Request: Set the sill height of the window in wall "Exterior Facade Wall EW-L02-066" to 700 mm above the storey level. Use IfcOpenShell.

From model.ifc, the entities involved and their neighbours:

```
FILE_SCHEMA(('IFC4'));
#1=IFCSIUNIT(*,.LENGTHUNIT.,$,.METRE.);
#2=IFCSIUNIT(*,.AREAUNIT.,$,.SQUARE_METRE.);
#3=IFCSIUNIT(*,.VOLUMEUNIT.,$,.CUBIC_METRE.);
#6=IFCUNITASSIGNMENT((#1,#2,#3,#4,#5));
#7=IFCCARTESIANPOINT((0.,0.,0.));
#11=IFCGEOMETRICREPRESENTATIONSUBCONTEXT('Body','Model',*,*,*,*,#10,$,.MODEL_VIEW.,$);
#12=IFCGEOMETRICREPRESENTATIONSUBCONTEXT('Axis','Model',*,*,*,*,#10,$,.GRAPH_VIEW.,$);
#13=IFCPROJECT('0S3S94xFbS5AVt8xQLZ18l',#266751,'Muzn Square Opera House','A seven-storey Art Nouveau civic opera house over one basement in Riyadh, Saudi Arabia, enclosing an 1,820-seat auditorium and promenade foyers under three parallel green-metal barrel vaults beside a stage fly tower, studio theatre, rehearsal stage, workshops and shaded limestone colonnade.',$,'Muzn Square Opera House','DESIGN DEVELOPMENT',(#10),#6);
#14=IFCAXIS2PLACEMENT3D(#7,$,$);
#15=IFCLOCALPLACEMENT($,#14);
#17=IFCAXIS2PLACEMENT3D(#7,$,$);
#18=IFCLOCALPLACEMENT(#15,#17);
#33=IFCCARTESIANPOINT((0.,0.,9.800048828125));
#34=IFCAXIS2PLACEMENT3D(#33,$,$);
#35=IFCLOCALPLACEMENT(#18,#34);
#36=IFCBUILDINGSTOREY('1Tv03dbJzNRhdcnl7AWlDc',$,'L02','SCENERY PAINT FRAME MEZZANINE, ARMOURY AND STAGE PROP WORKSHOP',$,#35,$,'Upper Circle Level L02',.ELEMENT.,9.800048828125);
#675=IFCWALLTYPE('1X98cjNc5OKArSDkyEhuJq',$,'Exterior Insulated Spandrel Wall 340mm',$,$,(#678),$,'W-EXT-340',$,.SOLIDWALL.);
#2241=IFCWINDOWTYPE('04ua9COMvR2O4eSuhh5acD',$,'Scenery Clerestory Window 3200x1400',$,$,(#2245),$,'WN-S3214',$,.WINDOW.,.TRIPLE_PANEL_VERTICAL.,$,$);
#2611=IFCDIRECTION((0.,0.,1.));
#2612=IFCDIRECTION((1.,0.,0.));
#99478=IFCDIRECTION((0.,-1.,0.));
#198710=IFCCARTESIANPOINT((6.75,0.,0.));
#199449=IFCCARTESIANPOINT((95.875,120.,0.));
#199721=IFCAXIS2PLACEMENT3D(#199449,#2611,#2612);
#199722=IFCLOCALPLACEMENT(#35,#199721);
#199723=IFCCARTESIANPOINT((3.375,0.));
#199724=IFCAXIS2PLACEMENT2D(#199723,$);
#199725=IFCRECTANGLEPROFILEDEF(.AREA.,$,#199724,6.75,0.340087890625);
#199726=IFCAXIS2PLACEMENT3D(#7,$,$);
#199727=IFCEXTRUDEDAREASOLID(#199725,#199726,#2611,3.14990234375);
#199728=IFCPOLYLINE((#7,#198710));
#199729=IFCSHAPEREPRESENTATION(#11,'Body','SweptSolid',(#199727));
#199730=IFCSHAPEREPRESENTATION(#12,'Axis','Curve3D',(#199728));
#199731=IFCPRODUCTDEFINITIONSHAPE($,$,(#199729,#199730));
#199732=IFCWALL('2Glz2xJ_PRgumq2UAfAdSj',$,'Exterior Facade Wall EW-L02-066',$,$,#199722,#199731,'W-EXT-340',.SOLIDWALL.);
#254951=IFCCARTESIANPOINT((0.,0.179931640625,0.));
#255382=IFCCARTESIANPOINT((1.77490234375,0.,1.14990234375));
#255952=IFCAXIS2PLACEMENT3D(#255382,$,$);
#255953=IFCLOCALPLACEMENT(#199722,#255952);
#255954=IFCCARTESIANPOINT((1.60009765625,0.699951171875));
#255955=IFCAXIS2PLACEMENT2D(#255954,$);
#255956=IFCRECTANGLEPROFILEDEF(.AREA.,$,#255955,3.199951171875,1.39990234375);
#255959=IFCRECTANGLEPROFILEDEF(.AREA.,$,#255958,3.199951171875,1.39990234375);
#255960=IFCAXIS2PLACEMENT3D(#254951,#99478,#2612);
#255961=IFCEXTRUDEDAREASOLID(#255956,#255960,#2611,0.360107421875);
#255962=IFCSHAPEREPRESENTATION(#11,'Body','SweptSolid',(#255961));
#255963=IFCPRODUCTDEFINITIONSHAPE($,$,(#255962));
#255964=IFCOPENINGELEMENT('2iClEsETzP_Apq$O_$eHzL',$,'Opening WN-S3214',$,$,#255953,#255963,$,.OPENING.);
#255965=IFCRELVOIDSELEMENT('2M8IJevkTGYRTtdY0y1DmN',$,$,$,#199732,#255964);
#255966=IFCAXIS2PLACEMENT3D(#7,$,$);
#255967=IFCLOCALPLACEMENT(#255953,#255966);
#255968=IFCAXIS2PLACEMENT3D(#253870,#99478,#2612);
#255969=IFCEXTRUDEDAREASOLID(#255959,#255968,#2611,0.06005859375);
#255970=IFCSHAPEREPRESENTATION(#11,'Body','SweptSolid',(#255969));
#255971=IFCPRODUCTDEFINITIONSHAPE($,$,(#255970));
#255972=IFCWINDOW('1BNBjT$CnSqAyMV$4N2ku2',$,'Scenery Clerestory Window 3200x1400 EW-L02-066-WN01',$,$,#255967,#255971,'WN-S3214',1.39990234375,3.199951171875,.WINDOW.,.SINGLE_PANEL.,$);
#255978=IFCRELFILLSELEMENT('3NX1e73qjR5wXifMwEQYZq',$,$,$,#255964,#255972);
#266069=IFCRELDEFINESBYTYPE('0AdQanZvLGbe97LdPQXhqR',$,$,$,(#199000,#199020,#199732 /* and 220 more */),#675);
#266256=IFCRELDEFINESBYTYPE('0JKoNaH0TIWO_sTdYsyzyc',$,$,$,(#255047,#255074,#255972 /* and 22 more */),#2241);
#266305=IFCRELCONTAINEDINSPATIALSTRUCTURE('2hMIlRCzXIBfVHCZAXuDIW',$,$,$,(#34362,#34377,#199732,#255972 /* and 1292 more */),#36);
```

```python
import numpy as np
import ifcopenshell
import ifcopenshell.api.geometry
import ifcopenshell.geom
import ifcopenshell.util.element
import ifcopenshell.util.placement
import ifcopenshell.util.shape
import ifcopenshell.util.unit

model = ifcopenshell.open("model.ifc")
unit_scale = ifcopenshell.util.unit.calculate_unit_scale(model)

window = model.by_guid("1BNBjT$CnSqAyMV$4N2ku2")
opening = window.FillsVoids[0].RelatingOpeningElement
storey = ifcopenshell.util.element.get_container(window, ifc_class="IfcBuildingStorey")
level = ifcopenshell.util.placement.get_local_placement(storey.ObjectPlacement)[2, 3]

# The opening's origin need not be at the sill, so measure its lowest point.
shape = ifcopenshell.geom.create_shape(ifcopenshell.geom.settings(), opening)
bottom = ifcopenshell.util.shape.get_shape_bottom_elevation(shape, shape.geometry) / unit_scale
dz = level + 0.7 / unit_scale - bottom

shift = np.array([0.0, 0.0, dz])
# The window is placed relative to its opening, so it follows when the opening moves.
matrix = ifcopenshell.util.placement.get_local_placement(opening.ObjectPlacement)
matrix[:3, 3] += shift
ifcopenshell.api.geometry.edit_object_placement(
    model, product=opening, matrix=matrix, is_si=False, should_transform_children=True
)

print(f"moved by {dz * unit_scale:+.3f} m")

model.write("model_updated.ifc")
```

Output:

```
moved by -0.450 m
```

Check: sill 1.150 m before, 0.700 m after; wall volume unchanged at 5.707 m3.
